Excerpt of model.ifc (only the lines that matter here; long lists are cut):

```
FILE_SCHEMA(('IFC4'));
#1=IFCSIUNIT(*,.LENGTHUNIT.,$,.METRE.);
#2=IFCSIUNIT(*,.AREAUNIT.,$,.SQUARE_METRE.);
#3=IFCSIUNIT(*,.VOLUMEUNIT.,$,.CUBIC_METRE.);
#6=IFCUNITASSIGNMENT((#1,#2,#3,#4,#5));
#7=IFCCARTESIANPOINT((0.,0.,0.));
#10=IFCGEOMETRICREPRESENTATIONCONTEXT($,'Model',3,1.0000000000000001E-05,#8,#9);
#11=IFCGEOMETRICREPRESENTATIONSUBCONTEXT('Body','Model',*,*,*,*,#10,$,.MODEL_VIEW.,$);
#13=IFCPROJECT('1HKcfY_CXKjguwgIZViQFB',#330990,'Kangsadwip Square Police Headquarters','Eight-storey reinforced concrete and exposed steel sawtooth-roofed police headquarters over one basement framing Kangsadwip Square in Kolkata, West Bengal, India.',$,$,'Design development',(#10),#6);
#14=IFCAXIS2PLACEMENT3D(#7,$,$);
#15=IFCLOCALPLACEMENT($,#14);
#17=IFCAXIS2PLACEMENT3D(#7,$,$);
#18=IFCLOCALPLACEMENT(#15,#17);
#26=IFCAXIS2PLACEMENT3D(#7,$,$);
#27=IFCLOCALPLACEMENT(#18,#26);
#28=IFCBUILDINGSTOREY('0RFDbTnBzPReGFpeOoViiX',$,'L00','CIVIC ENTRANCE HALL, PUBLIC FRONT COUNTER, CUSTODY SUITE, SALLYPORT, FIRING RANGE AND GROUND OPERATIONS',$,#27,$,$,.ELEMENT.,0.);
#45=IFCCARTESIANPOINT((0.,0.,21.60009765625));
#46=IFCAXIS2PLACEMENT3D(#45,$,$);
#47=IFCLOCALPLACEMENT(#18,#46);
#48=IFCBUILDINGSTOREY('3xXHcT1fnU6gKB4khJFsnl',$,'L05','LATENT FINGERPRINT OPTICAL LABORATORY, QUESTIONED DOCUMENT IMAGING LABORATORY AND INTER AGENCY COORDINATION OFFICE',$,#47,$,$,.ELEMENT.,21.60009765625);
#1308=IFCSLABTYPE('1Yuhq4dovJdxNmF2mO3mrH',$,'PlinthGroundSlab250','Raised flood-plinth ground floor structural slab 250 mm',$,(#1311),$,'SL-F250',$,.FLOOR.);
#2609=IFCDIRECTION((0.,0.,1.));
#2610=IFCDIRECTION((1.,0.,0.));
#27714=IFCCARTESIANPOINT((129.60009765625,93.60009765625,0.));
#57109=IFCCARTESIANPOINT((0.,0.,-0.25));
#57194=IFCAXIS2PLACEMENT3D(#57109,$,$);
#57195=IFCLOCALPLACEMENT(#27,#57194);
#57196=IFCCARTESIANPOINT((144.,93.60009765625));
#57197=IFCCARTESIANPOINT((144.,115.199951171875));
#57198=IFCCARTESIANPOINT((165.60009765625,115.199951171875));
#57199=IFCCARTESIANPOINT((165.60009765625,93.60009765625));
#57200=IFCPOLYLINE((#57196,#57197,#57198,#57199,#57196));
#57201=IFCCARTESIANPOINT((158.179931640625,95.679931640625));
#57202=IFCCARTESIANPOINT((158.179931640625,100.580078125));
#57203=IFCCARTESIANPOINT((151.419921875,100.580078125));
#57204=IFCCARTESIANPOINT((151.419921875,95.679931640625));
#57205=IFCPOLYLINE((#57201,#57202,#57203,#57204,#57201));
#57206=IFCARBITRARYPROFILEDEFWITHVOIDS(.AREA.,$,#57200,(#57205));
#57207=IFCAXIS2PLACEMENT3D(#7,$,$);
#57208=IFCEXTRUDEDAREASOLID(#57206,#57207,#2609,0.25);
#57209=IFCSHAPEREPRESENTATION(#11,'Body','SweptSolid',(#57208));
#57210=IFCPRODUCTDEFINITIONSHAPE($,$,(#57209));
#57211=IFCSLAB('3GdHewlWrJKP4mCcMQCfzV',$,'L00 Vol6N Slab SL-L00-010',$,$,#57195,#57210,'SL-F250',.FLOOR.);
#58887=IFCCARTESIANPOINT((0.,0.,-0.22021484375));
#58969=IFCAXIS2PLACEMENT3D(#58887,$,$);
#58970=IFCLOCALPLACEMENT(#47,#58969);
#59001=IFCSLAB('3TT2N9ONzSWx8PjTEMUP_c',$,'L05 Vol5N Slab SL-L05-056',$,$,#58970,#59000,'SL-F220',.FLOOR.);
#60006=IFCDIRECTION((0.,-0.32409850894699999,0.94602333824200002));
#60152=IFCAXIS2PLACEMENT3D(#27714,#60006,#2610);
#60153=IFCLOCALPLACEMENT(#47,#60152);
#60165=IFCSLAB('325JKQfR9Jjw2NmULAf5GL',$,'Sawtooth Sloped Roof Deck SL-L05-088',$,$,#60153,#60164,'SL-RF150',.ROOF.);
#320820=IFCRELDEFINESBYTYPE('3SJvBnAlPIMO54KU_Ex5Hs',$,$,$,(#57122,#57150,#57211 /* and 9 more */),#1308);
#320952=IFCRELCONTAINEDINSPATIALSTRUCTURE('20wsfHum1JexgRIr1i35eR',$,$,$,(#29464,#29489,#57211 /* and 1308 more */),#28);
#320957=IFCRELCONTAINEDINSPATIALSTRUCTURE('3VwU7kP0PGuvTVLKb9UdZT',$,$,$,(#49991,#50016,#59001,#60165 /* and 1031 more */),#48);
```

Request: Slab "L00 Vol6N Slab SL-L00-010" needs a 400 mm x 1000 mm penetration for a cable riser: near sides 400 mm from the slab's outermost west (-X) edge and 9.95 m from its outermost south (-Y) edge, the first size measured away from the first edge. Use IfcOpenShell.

```python
import numpy as np
import ifcopenshell
import ifcopenshell.api.feature
import ifcopenshell.api.geometry
import ifcopenshell.api.root
import ifcopenshell.geom
import ifcopenshell.util.placement
import ifcopenshell.util.representation
import ifcopenshell.util.shape
import ifcopenshell.util.unit

model = ifcopenshell.open("model.ifc")
unit_scale = ifcopenshell.util.unit.calculate_unit_scale(model)
settings = ifcopenshell.geom.settings()


def volume(element):
    """Net volume in cubic metres, openings subtracted."""
    shape = ifcopenshell.geom.create_shape(settings, element)
    return ifcopenshell.util.shape.get_volume(shape.geometry)


slab = model.by_guid("3GdHewlWrJKP4mCcMQCfzV")
before = volume(slab)

# Extent in the slab's own axes, in metres. The edges named are its -X and -Y sides.
slab_shape = ifcopenshell.geom.create_shape(settings, slab)
vertices = ifcopenshell.util.shape.get_vertices(slab_shape.geometry)
x_min, y_min, bottom = vertices.min(axis=0)
top = vertices[:, 2].max()

opening = ifcopenshell.api.root.create_entity(model, ifc_class="IfcOpeningElement", name="Cable riser opening", predefined_type="OPENING")
context = ifcopenshell.util.representation.get_context(model, "Model", "Body", "MODEL_VIEW")
width, depth = 0.4, 1
outline = [(0.0, 0.0), (width, 0.0), (width, depth), (0.0, depth), (0.0, 0.0)]
# Overshoot both faces by 50 mm so the cut is clean.
shape = ifcopenshell.api.geometry.add_slab_representation(
    model, context=context, depth=top - bottom + 0.1, polyline=outline
)
ifcopenshell.api.geometry.assign_representation(model, product=opening, representation=shape)

matrix = ifcopenshell.util.placement.get_local_placement(slab.ObjectPlacement)
matrix[:, 3] = matrix @ np.append(np.array([x_min + 0.4, y_min + 9.95, bottom - 0.05]) / unit_scale, 1.0)
ifcopenshell.api.geometry.edit_object_placement(model, product=opening, matrix=matrix, is_si=False)
ifcopenshell.api.feature.add_feature(model, feature=opening, element=slab)

after = volume(slab)

print(f"slab volume {before:.3f} -> {after:.3f} m3")

model.write("model-out.ifc")
```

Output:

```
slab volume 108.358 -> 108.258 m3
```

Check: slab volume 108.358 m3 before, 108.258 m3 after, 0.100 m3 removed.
